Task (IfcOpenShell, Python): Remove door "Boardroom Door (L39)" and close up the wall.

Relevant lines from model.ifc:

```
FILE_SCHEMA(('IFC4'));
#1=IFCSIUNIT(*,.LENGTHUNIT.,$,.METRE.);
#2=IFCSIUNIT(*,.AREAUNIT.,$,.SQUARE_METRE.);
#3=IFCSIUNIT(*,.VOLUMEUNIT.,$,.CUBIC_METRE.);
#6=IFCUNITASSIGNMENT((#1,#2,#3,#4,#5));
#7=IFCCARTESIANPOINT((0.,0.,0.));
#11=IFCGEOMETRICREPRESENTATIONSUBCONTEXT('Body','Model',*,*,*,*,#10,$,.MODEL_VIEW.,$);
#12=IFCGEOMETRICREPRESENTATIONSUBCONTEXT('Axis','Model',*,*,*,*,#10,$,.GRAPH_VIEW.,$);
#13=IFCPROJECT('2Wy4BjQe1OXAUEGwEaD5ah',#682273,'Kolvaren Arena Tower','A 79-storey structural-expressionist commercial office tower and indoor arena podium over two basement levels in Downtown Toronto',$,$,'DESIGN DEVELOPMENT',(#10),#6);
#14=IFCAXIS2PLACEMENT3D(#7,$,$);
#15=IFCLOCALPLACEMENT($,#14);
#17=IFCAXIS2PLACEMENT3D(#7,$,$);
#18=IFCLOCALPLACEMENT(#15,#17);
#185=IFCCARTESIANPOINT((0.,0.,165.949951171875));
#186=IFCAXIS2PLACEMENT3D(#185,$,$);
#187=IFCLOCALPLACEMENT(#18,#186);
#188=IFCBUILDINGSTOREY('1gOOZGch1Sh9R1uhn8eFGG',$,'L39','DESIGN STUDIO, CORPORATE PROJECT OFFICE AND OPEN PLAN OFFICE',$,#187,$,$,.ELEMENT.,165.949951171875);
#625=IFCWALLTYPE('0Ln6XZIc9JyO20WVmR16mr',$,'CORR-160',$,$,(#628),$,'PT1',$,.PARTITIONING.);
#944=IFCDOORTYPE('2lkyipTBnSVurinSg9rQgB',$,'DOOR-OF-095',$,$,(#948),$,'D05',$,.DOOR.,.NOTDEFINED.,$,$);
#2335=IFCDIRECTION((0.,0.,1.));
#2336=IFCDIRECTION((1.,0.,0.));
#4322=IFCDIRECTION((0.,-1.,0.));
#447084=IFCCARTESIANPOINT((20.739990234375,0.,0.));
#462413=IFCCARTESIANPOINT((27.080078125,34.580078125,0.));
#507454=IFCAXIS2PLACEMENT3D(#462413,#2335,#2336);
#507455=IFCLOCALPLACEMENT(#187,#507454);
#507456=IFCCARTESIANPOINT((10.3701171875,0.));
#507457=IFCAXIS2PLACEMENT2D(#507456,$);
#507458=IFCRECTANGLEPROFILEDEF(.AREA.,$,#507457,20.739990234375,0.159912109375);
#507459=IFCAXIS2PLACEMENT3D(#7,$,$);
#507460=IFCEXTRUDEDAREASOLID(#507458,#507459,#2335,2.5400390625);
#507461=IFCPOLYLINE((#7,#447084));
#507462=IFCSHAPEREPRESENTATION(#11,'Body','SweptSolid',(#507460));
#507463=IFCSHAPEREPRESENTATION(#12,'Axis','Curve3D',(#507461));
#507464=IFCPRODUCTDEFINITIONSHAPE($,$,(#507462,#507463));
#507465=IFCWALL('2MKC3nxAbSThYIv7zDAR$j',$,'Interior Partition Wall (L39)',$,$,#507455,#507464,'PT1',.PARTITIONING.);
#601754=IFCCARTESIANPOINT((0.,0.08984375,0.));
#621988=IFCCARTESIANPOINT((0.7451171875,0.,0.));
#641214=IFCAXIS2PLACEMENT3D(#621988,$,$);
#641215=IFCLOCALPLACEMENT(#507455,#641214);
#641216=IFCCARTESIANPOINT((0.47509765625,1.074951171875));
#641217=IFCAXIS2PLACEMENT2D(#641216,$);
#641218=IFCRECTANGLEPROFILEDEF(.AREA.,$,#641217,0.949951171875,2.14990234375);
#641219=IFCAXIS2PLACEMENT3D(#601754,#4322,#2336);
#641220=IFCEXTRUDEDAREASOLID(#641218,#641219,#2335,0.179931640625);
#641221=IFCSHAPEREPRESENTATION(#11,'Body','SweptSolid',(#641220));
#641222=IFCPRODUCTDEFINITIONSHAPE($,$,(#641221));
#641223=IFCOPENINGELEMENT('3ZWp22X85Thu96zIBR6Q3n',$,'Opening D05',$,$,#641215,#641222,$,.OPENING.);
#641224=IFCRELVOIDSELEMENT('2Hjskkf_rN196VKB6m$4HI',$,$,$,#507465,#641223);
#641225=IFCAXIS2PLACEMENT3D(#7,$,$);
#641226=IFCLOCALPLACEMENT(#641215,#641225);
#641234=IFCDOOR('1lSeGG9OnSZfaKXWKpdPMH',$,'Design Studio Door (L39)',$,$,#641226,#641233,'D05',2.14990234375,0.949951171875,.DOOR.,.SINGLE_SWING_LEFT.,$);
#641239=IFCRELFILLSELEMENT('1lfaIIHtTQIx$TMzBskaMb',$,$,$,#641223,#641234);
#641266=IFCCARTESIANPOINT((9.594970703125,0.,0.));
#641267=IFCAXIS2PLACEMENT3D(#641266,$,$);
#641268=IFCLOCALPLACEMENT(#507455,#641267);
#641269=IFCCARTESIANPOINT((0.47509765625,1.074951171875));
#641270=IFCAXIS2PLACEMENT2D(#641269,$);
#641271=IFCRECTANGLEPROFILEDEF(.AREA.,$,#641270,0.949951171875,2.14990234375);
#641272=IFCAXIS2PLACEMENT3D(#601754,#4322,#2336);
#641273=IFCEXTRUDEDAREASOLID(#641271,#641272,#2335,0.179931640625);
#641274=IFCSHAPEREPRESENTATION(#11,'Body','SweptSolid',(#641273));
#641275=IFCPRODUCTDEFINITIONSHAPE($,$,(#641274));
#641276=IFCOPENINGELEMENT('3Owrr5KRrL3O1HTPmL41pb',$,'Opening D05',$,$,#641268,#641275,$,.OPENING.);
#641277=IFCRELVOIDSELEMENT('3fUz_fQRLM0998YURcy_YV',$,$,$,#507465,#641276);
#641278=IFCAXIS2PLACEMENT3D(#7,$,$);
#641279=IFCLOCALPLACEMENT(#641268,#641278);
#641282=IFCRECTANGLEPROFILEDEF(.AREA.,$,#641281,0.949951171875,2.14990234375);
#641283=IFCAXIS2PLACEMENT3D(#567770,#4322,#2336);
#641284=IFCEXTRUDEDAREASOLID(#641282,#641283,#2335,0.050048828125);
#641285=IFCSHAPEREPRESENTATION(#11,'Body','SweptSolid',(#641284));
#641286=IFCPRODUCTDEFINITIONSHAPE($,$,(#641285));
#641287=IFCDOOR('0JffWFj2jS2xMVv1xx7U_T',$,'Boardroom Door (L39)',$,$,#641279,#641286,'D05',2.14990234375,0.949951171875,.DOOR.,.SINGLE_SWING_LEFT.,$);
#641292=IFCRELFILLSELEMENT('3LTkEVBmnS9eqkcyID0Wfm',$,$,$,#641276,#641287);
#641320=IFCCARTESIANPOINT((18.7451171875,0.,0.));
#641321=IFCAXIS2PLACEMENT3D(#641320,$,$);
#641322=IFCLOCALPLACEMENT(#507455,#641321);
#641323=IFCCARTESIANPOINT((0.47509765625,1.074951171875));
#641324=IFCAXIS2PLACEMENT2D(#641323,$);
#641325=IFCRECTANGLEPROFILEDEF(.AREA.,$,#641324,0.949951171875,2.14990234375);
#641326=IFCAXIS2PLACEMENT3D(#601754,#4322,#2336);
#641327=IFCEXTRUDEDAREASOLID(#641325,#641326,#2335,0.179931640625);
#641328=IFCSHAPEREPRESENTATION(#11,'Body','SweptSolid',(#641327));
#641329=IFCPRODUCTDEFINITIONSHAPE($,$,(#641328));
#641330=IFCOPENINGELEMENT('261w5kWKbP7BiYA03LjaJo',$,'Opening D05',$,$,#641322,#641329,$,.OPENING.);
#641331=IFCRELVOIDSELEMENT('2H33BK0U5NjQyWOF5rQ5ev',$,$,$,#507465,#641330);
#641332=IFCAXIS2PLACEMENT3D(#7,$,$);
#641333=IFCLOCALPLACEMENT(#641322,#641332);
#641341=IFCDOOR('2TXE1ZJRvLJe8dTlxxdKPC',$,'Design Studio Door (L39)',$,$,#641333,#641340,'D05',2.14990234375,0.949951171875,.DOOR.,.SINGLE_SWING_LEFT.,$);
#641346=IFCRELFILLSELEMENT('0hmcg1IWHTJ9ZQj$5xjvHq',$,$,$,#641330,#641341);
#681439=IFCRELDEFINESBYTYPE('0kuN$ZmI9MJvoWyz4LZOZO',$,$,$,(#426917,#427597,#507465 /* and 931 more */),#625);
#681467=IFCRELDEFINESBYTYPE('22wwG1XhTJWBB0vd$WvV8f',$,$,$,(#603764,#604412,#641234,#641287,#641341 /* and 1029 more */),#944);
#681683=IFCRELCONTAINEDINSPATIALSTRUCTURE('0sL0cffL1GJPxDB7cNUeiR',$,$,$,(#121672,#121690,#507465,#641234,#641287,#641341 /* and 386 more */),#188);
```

```python
import ifcopenshell
import ifcopenshell.api.feature
import ifcopenshell.api.root
import ifcopenshell.geom
import ifcopenshell.util.shape

model = ifcopenshell.open("model.ifc")
settings = ifcopenshell.geom.settings()


def volume(element):
    """Net volume in cubic metres, openings subtracted."""
    shape = ifcopenshell.geom.create_shape(settings, element)
    return ifcopenshell.util.shape.get_volume(shape.geometry)


door = model.by_guid("0JffWFj2jS2xMVv1xx7U_T")
opening = door.FillsVoids[0].RelatingOpeningElement
wall = opening.VoidsElements[0].RelatingBuildingElement
before = volume(wall)

ifcopenshell.api.root.remove_product(model, product=door)
ifcopenshell.api.feature.remove_feature(model, feature=opening)

after = volume(wall)

print(f"wall volume {before:.3f} -> {after:.3f} m3")

model.write("model_rev.ifc")
```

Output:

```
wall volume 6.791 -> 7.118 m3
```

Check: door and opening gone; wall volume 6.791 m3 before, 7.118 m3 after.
